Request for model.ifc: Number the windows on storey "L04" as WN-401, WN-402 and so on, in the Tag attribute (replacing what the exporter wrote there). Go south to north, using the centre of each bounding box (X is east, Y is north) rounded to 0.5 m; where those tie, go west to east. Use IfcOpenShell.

First a look at what the model holds.

```python
import ifcopenshell
import ifcopenshell.util.element
import ifcopenshell.util.placement

model = ifcopenshell.open("model.ifc")
print(model.schema)
storey = next(s for s in model.by_type("IfcBuildingStorey") if s.Name == "L04")
windows = [e for e in ifcopenshell.util.element.get_decomposition(storey) if e.is_a("IfcWindow")]
for e in sorted(windows, key=lambda e: e.id()):
    origin = ifcopenshell.util.placement.get_local_placement(e.ObjectPlacement)[:3, 3]
    print(e.id(), e.Tag, e.Name, origin.round(2) + 0.0, sep=" | ")
```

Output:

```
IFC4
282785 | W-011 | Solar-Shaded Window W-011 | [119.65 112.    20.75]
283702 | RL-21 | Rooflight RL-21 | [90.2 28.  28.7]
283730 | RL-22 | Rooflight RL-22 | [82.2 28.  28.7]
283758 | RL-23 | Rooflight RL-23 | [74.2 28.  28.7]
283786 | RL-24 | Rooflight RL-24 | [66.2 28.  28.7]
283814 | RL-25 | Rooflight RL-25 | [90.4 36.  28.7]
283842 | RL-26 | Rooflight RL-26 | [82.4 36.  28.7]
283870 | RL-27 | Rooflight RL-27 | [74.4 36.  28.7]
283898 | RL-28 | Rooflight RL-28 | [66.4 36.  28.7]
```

```python
import ifcopenshell
import ifcopenshell.geom
import ifcopenshell.util.element
import ifcopenshell.util.shape

model = ifcopenshell.open("model.ifc")
settings = ifcopenshell.geom.settings()
settings.set("use-world-coords", True)


def centre(element):
    shape = ifcopenshell.geom.create_shape(settings, element)
    return ifcopenshell.util.shape.get_bbox_centroid(shape.geometry)


storey = next(s for s in model.by_type("IfcBuildingStorey") if s.Name == "L04")
windows = [e for e in ifcopenshell.util.element.get_decomposition(storey) if e.is_a("IfcWindow")]

# Insertion points can sit at a corner or the storey origin, so sort by the geometry (in metres).
centres = {e: centre(e) for e in windows}
windows.sort(key=lambda e: (round(centres[e][1] / 0.5), centres[e][0]))

for i, e in enumerate(windows, start=1):
    number = f"WN-4{i:02d}"
    e.Tag = number
    print(e.id(), number)

model.write("model_edited.ifc")
```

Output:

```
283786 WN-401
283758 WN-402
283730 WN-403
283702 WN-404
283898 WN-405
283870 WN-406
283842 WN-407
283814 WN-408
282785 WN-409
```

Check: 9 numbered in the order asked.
